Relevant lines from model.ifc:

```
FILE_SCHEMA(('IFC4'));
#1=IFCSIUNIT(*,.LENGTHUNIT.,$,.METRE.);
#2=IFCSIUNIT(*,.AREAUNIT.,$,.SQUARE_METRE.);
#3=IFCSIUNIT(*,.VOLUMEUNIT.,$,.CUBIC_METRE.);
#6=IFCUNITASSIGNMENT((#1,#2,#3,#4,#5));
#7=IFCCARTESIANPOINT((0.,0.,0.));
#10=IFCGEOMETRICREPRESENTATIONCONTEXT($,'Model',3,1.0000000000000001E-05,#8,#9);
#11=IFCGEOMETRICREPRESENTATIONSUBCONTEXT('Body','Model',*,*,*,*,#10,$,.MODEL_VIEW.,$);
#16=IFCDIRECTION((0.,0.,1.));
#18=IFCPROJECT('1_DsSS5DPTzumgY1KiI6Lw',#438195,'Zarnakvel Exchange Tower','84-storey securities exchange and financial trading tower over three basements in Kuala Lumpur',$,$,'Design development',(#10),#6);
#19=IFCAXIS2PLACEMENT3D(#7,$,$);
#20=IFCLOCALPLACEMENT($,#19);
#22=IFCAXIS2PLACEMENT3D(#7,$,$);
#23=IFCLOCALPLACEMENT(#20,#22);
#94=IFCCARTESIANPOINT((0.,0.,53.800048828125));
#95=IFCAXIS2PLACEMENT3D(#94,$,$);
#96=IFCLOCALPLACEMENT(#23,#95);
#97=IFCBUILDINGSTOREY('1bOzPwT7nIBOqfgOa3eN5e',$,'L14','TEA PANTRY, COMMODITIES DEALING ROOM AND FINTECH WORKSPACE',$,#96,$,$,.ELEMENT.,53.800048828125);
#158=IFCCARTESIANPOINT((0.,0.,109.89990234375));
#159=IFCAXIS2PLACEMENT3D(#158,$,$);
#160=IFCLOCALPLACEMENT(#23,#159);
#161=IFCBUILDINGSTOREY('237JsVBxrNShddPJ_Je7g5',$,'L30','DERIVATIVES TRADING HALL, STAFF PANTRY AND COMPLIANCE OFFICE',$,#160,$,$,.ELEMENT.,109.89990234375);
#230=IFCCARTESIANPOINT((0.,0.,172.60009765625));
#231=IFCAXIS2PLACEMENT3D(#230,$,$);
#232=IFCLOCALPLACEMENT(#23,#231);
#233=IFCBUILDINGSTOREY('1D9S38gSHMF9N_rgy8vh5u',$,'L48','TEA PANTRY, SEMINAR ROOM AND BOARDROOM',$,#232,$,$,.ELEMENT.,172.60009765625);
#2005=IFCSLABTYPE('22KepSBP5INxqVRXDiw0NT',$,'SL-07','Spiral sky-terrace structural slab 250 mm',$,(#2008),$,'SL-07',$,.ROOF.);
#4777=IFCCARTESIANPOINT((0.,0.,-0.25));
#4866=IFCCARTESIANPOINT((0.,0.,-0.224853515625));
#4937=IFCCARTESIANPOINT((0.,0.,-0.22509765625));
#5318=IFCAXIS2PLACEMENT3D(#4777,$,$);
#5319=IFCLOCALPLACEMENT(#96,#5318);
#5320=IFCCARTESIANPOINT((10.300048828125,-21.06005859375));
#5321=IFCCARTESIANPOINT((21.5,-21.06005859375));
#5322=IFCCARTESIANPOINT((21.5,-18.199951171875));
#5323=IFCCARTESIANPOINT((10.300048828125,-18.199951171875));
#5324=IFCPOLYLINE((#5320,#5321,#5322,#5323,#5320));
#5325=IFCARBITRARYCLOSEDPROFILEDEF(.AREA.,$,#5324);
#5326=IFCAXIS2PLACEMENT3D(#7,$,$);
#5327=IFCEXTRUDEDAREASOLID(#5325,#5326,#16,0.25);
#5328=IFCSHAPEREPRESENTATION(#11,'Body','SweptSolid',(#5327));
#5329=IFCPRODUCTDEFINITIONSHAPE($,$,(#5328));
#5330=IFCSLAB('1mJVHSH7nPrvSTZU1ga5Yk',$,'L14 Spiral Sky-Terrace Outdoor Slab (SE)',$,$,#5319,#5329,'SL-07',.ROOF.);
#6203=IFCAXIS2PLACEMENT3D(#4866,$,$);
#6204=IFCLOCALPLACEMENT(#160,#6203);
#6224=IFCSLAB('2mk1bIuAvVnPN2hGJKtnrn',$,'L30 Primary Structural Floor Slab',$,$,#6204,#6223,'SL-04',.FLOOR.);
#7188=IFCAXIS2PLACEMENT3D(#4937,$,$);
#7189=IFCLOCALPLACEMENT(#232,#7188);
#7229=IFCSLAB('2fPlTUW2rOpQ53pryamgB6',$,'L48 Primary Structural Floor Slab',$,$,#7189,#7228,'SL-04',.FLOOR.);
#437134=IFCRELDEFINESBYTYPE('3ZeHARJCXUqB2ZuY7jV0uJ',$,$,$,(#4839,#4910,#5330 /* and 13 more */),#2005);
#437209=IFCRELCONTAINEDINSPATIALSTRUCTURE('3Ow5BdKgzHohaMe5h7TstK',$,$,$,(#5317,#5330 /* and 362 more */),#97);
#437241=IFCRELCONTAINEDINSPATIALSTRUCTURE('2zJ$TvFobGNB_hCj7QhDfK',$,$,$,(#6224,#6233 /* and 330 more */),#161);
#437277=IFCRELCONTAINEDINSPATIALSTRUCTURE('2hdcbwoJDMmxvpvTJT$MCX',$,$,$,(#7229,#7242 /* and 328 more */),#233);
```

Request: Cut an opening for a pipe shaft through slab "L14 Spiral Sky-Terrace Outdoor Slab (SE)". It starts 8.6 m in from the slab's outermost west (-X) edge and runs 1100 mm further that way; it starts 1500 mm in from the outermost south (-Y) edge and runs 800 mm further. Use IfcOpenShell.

```python
import numpy as np
import ifcopenshell
import ifcopenshell.api.feature
import ifcopenshell.api.geometry
import ifcopenshell.api.root
import ifcopenshell.geom
import ifcopenshell.util.placement
import ifcopenshell.util.representation
import ifcopenshell.util.shape
import ifcopenshell.util.unit

model = ifcopenshell.open("model.ifc")
unit_scale = ifcopenshell.util.unit.calculate_unit_scale(model)
settings = ifcopenshell.geom.settings()


def volume(element):
    """Net volume in cubic metres, openings subtracted."""
    shape = ifcopenshell.geom.create_shape(settings, element)
    return ifcopenshell.util.shape.get_volume(shape.geometry)


slab = model.by_id(5330)
before = volume(slab)

# Extent in the slab's own axes, in metres. The edges named are its -X and -Y sides.
slab_shape = ifcopenshell.geom.create_shape(settings, slab)
vertices = ifcopenshell.util.shape.get_vertices(slab_shape.geometry)
x_min, y_min, bottom = vertices.min(axis=0)
top = vertices[:, 2].max()

opening = ifcopenshell.api.root.create_entity(model, ifc_class="IfcOpeningElement", name="Pipe shaft opening", predefined_type="OPENING")
context = ifcopenshell.util.representation.get_context(model, "Model", "Body", "MODEL_VIEW")
width, depth = 1.1, 0.8
outline = [(0.0, 0.0), (width, 0.0), (width, depth), (0.0, depth), (0.0, 0.0)]
# Overshoot both faces by 50 mm so the cut is clean.
shape = ifcopenshell.api.geometry.add_slab_representation(
    model, context=context, depth=top - bottom + 0.1, polyline=outline
)
ifcopenshell.api.geometry.assign_representation(model, product=opening, representation=shape)

matrix = ifcopenshell.util.placement.get_local_placement(slab.ObjectPlacement)
matrix[:, 3] = matrix @ np.append(np.array([x_min + 8.6, y_min + 1.5, bottom - 0.05]) / unit_scale, 1.0)
ifcopenshell.api.geometry.edit_object_placement(model, product=opening, matrix=matrix, is_si=False)
ifcopenshell.api.feature.add_feature(model, feature=opening, element=slab)

after = volume(slab)

print(f"slab volume {before:.3f} -> {after:.3f} m3")

model.write("model-out.ifc")
```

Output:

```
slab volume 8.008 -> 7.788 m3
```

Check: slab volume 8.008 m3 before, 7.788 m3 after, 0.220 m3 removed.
